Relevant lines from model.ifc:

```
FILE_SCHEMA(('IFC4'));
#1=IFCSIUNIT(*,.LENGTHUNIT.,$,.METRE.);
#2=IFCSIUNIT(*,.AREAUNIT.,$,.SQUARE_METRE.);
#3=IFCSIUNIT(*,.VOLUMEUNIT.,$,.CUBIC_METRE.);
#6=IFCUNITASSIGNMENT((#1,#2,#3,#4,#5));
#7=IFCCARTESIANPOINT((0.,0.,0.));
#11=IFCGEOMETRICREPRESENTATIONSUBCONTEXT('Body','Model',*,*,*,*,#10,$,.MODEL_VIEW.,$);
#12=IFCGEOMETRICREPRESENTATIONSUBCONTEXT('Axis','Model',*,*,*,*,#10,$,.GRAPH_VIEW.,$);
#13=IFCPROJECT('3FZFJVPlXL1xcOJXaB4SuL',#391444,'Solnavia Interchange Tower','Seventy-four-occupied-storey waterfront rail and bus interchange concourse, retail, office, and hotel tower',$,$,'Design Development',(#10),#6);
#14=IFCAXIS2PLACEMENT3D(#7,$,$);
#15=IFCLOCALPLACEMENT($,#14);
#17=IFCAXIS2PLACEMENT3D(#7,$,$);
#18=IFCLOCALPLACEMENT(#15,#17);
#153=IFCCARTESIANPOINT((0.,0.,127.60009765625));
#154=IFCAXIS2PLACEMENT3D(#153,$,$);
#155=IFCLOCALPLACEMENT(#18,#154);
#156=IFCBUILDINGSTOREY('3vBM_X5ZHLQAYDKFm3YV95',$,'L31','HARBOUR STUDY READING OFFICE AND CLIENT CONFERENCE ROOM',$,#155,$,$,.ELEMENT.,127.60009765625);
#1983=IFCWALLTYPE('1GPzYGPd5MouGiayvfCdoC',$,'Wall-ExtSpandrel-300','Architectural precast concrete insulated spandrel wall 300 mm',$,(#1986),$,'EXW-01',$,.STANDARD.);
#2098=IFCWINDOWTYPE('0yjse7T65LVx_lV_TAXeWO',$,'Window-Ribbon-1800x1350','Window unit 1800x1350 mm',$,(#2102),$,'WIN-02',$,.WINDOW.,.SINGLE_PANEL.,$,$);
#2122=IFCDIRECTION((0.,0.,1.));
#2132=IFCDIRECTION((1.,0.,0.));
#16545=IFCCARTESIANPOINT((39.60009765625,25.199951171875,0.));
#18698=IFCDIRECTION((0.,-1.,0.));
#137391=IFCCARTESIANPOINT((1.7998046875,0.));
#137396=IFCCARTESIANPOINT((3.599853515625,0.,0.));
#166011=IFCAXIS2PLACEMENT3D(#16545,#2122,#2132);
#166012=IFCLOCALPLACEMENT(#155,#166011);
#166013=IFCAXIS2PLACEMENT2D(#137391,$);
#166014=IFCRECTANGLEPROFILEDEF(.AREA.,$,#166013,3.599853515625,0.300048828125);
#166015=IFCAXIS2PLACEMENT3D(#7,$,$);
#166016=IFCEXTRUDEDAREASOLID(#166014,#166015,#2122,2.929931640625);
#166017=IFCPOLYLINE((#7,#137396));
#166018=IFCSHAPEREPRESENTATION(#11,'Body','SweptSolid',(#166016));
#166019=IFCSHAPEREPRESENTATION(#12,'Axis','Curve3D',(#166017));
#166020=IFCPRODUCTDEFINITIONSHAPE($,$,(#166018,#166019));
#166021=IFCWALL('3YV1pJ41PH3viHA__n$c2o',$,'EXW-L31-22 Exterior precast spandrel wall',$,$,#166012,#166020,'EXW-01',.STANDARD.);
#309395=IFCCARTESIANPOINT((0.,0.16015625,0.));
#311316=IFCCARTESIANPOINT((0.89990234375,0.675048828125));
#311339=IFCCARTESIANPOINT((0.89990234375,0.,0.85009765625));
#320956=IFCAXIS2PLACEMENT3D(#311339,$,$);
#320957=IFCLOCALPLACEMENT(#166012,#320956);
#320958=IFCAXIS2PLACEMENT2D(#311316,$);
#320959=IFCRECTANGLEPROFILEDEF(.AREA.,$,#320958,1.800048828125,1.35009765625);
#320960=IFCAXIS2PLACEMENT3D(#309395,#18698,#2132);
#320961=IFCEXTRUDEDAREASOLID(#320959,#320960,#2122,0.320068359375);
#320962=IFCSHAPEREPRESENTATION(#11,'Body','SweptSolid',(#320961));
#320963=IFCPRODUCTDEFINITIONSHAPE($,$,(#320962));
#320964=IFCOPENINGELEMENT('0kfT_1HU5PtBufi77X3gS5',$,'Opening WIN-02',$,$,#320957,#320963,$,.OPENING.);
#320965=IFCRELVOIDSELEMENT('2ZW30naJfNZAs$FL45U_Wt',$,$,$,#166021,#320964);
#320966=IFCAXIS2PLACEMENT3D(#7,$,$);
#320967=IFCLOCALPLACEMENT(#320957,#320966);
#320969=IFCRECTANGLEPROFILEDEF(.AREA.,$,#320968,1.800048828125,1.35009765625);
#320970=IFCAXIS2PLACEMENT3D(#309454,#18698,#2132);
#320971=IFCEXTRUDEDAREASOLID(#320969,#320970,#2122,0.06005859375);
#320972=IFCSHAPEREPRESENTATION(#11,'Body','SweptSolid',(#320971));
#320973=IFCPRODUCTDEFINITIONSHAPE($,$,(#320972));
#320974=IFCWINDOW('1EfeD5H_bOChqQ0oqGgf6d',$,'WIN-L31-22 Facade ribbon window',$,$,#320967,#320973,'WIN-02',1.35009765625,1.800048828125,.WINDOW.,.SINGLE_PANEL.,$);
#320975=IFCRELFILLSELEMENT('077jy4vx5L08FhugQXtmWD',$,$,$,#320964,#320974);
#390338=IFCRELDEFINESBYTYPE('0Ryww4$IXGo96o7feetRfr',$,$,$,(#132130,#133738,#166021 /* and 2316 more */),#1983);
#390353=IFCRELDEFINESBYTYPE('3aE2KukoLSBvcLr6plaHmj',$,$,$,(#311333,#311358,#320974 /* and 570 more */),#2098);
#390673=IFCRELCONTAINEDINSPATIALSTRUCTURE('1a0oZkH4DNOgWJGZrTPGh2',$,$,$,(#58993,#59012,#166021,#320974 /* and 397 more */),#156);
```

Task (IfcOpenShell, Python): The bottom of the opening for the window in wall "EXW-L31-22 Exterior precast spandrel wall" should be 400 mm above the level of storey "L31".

```python
import numpy as np
import ifcopenshell
import ifcopenshell.api.geometry
import ifcopenshell.geom
import ifcopenshell.util.element
import ifcopenshell.util.placement
import ifcopenshell.util.shape
import ifcopenshell.util.unit

model = ifcopenshell.open("model.ifc")
unit_scale = ifcopenshell.util.unit.calculate_unit_scale(model)

window = model.by_guid("1EfeD5H_bOChqQ0oqGgf6d")
opening = window.FillsVoids[0].RelatingOpeningElement
storey = ifcopenshell.util.element.get_container(window, ifc_class="IfcBuildingStorey")
level = ifcopenshell.util.placement.get_local_placement(storey.ObjectPlacement)[2, 3]

# The opening's origin need not be at the sill, so measure its lowest point.
shape = ifcopenshell.geom.create_shape(ifcopenshell.geom.settings(), opening)
bottom = ifcopenshell.util.shape.get_shape_bottom_elevation(shape, shape.geometry) / unit_scale
dz = level + 0.4 / unit_scale - bottom

shift = np.array([0.0, 0.0, dz])
# The window is placed relative to its opening, so it follows when the opening moves.
matrix = ifcopenshell.util.placement.get_local_placement(opening.ObjectPlacement)
matrix[:3, 3] += shift
ifcopenshell.api.geometry.edit_object_placement(
    model, product=opening, matrix=matrix, is_si=False, should_transform_children=True
)

print(f"moved by {dz * unit_scale:+.3f} m")

model.write("model_updated.ifc")
```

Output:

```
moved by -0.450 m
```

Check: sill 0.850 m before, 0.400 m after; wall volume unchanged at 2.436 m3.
